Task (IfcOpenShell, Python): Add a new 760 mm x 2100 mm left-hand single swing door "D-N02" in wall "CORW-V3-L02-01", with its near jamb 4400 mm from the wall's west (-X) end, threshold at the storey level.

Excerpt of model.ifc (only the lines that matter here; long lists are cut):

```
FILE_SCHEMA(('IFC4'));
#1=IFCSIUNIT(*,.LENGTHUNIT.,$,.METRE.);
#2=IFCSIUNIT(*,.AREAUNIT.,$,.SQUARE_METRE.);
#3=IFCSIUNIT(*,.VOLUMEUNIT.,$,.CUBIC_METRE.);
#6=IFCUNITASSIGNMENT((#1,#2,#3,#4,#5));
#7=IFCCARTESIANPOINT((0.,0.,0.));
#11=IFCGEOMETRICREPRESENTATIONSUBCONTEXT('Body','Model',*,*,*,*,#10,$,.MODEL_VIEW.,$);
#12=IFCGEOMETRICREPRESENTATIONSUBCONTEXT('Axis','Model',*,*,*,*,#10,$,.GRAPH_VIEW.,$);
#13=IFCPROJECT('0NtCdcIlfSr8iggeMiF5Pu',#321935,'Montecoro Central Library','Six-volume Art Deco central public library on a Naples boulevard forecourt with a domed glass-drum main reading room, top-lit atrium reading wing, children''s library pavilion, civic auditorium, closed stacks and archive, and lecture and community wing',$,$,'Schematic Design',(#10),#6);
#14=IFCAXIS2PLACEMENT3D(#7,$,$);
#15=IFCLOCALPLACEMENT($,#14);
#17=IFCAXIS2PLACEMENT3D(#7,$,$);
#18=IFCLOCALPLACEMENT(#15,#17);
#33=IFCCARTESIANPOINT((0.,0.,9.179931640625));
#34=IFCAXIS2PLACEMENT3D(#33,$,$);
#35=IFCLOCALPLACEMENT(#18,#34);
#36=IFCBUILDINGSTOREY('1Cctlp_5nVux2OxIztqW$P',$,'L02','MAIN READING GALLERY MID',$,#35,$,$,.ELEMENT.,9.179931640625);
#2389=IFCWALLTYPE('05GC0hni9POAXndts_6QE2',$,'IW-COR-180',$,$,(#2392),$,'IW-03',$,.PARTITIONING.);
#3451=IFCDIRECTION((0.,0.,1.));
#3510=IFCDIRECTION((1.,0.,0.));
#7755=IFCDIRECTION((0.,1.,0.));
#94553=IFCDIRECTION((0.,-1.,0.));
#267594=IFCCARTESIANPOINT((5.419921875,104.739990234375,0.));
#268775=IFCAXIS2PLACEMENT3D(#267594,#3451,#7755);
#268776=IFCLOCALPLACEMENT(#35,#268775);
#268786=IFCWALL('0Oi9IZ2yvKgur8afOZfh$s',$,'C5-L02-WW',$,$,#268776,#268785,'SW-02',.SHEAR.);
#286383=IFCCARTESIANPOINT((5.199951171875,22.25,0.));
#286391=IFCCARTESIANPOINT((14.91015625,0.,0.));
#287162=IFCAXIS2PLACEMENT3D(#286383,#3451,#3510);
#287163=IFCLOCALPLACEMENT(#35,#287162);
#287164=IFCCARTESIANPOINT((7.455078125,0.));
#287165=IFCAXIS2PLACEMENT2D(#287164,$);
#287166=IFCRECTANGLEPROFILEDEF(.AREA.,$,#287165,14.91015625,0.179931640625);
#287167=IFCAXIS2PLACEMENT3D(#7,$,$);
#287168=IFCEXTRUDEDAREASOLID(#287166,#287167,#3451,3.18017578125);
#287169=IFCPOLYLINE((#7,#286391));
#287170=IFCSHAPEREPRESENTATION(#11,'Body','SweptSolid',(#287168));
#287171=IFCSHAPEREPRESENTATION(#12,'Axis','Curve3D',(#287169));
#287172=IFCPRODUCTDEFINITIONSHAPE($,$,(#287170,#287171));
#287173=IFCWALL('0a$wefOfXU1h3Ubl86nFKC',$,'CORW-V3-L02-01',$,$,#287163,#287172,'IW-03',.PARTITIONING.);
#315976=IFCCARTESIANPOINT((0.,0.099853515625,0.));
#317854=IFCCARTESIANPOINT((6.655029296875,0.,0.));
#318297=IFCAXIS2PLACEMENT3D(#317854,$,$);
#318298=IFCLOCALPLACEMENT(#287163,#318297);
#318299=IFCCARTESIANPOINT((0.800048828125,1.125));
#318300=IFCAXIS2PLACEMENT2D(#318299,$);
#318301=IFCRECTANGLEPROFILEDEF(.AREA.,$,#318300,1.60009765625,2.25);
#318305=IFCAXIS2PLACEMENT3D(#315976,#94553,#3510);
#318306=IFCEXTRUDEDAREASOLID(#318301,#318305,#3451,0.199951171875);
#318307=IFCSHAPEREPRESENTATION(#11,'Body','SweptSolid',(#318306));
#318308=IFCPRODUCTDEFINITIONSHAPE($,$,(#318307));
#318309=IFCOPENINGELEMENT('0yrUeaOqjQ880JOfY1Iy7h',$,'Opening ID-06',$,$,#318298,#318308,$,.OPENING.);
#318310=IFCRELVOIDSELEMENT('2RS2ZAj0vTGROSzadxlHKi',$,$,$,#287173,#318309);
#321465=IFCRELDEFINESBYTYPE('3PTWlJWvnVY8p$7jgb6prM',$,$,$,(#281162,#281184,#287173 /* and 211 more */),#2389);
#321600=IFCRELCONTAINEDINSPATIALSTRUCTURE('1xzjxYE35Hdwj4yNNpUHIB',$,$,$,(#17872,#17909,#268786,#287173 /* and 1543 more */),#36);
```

```python
import numpy as np
import ifcopenshell
import ifcopenshell.api.feature
import ifcopenshell.api.geometry
import ifcopenshell.api.root
import ifcopenshell.api.spatial
import ifcopenshell.geom
import ifcopenshell.util.element
import ifcopenshell.util.placement
import ifcopenshell.util.representation
import ifcopenshell.util.shape
import ifcopenshell.util.unit

model = ifcopenshell.open("model.ifc")
unit_scale = ifcopenshell.util.unit.calculate_unit_scale(model)
settings = ifcopenshell.geom.settings()


def volume(element):
    """Net volume in cubic metres, openings subtracted."""
    shape = ifcopenshell.geom.create_shape(settings, element)
    return ifcopenshell.util.shape.get_volume(shape.geometry)


wall = model.by_guid("0a$wefOfXU1h3Ubl86nFKC")
storey = ifcopenshell.util.element.get_container(wall, ifc_class="IfcBuildingStorey")
context = ifcopenshell.util.representation.get_context(model, "Model", "Body", "MODEL_VIEW")
before = volume(wall)

width, height, from_end, sill = 0.76, 2.1, 4.4, 0.0  # metres

# The wall runs along its own X axis, and the end named is its -X end.
wall_shape = ifcopenshell.geom.create_shape(settings, wall)
x, y, z = ifcopenshell.util.shape.get_vertices(wall_shape.geometry).T
start = x.min() + from_end
face, thickness = float(y.min()), float(y.max() - y.min())
wall_matrix = ifcopenshell.util.placement.get_local_placement(wall.ObjectPlacement)
level = ifcopenshell.util.placement.get_local_placement(storey.ObjectPlacement)[2, 3]


def in_wall(x, y):
    """Placement at x, y metres in the wall's axes, at sill height."""
    matrix = wall_matrix.copy()
    matrix[:, 3] = wall_matrix @ np.array([x / unit_scale, y / unit_scale, 0.0, 1.0])
    matrix[2, 3] = level + sill / unit_scale
    return matrix


# Opening: a box that overshoots both wall faces by 50 mm.
opening = ifcopenshell.api.root.create_entity(model, ifc_class="IfcOpeningElement", predefined_type="OPENING")
box = ifcopenshell.api.geometry.add_wall_representation(
    model, context=context, length=width, height=height, thickness=thickness + 0.1
)
ifcopenshell.api.geometry.assign_representation(model, product=opening, representation=box)
ifcopenshell.api.geometry.edit_object_placement(model, product=opening, matrix=in_wall(start, face - 0.05), is_si=False)
ifcopenshell.api.feature.add_feature(model, feature=opening, element=wall)

door = ifcopenshell.api.root.create_entity(model, ifc_class="IfcDoor", name="D-N02", predefined_type="DOOR")
door.OverallWidth, door.OverallHeight = width / unit_scale, height / unit_scale
door.OperationType = "SINGLE_SWING_LEFT"
body = ifcopenshell.api.geometry.add_door_representation(
    model,
    context=context,
    overall_width=door.OverallWidth,
    overall_height=door.OverallHeight,
    operation_type="SINGLE_SWING_LEFT",
    lining_properties={"LiningDepth": thickness / unit_scale, "ThresholdDepth": thickness / unit_scale},
)
ifcopenshell.api.geometry.assign_representation(model, product=door, representation=body)
ifcopenshell.api.spatial.assign_container(model, products=[door], relating_structure=storey)
ifcopenshell.api.feature.add_filling(model, opening=opening, element=door)

# The lining spans the wall, so the door starts at the wall face.
ifcopenshell.api.geometry.edit_object_placement(model, product=door, matrix=in_wall(start, face), is_si=False)

after = volume(wall)

print(f"wall volume {before:.3f} -> {after:.3f} m3")

model.write("model_edited.ifc")
```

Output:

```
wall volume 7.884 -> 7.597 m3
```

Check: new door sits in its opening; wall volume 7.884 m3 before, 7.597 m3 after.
